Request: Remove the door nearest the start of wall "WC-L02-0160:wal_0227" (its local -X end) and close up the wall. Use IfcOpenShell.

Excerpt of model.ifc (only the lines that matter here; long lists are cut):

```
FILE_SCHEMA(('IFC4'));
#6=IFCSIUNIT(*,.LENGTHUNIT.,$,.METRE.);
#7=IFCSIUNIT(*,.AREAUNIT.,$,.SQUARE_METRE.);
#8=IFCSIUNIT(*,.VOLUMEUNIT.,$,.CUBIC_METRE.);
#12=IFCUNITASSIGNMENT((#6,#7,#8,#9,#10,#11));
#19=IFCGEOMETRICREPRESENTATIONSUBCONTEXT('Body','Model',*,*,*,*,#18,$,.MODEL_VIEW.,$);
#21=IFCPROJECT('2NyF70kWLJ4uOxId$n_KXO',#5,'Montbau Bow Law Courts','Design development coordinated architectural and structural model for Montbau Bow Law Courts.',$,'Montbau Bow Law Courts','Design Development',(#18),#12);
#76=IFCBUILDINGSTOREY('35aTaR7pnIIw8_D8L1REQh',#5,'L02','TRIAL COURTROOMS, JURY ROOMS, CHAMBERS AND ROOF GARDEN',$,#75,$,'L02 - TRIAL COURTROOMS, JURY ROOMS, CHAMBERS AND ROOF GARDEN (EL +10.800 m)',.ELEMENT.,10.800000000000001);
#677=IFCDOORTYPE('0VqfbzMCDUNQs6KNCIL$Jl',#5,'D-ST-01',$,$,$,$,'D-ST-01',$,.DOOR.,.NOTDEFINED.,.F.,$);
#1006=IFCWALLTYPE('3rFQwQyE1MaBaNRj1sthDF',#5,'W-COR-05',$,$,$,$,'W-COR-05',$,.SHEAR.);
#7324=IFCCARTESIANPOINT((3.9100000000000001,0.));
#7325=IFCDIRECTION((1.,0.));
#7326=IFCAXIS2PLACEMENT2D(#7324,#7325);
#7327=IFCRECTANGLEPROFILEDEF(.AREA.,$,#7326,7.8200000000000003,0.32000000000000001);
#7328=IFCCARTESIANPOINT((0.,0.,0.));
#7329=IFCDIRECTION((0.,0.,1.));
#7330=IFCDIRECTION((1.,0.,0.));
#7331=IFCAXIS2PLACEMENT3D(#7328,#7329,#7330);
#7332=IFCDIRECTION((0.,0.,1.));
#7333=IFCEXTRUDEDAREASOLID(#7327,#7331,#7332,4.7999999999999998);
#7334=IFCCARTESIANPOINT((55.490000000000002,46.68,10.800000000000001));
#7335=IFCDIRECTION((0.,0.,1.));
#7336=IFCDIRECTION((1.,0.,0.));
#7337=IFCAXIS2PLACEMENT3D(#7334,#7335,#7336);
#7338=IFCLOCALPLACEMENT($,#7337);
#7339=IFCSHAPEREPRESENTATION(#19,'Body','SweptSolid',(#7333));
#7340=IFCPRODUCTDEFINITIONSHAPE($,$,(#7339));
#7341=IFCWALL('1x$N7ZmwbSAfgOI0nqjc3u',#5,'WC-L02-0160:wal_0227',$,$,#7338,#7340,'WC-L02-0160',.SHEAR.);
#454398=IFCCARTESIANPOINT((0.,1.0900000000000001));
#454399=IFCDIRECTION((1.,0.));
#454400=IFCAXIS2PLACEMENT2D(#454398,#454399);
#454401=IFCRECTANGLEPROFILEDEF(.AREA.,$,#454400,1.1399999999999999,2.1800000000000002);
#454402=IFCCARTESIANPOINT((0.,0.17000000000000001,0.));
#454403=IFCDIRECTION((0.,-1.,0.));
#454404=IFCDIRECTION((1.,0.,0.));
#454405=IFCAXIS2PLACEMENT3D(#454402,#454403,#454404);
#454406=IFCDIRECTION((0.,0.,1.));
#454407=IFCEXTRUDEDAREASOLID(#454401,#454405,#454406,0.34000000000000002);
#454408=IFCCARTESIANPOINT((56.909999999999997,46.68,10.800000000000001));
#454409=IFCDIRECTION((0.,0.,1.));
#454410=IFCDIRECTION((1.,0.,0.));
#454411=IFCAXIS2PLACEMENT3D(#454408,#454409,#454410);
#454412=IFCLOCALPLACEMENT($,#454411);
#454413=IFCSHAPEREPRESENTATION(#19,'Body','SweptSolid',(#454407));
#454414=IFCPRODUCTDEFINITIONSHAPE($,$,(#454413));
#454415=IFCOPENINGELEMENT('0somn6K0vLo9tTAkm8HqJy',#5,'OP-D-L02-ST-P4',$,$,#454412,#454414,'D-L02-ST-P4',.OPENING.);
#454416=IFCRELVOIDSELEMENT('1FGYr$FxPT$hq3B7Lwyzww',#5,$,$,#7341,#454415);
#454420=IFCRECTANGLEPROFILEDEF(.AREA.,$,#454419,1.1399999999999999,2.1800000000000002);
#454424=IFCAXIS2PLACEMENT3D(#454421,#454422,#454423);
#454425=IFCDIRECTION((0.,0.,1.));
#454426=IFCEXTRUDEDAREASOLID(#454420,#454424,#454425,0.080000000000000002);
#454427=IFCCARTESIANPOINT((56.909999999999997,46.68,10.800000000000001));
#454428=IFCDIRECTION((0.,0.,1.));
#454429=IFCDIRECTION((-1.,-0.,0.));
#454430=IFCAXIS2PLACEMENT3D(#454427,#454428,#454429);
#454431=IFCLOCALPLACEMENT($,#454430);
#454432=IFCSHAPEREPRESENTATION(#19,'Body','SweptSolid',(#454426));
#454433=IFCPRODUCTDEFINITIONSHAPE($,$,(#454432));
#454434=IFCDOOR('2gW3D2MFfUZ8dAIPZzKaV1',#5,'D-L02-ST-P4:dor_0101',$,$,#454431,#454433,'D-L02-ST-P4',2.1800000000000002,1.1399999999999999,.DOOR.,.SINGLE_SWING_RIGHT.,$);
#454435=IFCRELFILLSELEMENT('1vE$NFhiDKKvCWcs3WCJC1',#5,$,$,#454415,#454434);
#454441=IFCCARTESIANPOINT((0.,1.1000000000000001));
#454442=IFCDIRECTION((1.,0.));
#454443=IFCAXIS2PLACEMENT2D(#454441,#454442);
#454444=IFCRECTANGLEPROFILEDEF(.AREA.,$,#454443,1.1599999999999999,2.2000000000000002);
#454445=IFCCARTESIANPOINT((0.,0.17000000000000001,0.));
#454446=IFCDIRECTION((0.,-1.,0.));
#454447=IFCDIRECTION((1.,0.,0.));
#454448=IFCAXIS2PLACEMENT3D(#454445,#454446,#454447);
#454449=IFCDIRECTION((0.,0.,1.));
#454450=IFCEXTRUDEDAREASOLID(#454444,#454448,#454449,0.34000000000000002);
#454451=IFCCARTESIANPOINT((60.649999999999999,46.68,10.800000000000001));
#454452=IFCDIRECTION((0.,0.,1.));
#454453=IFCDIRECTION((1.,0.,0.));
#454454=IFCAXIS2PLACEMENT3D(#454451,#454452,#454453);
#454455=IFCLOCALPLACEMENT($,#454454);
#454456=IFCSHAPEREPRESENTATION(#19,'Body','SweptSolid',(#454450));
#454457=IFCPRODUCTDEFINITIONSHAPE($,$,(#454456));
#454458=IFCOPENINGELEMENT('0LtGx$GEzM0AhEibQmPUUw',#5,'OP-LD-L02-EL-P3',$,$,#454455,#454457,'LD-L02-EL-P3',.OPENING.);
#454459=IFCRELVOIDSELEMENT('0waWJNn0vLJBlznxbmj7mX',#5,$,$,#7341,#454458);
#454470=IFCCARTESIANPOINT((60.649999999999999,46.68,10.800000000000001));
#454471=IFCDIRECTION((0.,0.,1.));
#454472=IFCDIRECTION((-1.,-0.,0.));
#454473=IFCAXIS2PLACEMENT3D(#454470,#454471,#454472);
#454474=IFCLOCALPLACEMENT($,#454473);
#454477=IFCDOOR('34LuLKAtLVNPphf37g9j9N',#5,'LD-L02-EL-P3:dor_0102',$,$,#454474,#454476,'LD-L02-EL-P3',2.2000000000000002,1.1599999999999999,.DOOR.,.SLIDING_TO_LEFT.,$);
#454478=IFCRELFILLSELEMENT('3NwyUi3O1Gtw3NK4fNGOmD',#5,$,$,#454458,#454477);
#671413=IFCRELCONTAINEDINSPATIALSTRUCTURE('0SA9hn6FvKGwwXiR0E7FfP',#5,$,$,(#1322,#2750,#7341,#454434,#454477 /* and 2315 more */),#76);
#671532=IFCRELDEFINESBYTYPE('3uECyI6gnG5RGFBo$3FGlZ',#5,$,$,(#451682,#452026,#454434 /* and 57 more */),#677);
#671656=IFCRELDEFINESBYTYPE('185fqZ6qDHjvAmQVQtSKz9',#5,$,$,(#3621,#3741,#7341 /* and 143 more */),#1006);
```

```python
import ifcopenshell
import ifcopenshell.api.feature
import ifcopenshell.api.root
import ifcopenshell.geom
import ifcopenshell.util.shape

model = ifcopenshell.open("model.ifc")
settings = ifcopenshell.geom.settings()


def volume(element):
    """Net volume in cubic metres, openings subtracted."""
    shape = ifcopenshell.geom.create_shape(settings, element)
    return ifcopenshell.util.shape.get_volume(shape.geometry)


door = model.by_id(454434)
opening = door.FillsVoids[0].RelatingOpeningElement
wall = opening.VoidsElements[0].RelatingBuildingElement
before = volume(wall)

ifcopenshell.api.root.remove_product(model, product=door)
ifcopenshell.api.feature.remove_feature(model, feature=opening)

after = volume(wall)

print(f"wall volume {before:.3f} -> {after:.3f} m3")

model.write("model-out.ifc")
```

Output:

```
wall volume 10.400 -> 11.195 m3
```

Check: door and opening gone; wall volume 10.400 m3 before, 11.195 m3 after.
